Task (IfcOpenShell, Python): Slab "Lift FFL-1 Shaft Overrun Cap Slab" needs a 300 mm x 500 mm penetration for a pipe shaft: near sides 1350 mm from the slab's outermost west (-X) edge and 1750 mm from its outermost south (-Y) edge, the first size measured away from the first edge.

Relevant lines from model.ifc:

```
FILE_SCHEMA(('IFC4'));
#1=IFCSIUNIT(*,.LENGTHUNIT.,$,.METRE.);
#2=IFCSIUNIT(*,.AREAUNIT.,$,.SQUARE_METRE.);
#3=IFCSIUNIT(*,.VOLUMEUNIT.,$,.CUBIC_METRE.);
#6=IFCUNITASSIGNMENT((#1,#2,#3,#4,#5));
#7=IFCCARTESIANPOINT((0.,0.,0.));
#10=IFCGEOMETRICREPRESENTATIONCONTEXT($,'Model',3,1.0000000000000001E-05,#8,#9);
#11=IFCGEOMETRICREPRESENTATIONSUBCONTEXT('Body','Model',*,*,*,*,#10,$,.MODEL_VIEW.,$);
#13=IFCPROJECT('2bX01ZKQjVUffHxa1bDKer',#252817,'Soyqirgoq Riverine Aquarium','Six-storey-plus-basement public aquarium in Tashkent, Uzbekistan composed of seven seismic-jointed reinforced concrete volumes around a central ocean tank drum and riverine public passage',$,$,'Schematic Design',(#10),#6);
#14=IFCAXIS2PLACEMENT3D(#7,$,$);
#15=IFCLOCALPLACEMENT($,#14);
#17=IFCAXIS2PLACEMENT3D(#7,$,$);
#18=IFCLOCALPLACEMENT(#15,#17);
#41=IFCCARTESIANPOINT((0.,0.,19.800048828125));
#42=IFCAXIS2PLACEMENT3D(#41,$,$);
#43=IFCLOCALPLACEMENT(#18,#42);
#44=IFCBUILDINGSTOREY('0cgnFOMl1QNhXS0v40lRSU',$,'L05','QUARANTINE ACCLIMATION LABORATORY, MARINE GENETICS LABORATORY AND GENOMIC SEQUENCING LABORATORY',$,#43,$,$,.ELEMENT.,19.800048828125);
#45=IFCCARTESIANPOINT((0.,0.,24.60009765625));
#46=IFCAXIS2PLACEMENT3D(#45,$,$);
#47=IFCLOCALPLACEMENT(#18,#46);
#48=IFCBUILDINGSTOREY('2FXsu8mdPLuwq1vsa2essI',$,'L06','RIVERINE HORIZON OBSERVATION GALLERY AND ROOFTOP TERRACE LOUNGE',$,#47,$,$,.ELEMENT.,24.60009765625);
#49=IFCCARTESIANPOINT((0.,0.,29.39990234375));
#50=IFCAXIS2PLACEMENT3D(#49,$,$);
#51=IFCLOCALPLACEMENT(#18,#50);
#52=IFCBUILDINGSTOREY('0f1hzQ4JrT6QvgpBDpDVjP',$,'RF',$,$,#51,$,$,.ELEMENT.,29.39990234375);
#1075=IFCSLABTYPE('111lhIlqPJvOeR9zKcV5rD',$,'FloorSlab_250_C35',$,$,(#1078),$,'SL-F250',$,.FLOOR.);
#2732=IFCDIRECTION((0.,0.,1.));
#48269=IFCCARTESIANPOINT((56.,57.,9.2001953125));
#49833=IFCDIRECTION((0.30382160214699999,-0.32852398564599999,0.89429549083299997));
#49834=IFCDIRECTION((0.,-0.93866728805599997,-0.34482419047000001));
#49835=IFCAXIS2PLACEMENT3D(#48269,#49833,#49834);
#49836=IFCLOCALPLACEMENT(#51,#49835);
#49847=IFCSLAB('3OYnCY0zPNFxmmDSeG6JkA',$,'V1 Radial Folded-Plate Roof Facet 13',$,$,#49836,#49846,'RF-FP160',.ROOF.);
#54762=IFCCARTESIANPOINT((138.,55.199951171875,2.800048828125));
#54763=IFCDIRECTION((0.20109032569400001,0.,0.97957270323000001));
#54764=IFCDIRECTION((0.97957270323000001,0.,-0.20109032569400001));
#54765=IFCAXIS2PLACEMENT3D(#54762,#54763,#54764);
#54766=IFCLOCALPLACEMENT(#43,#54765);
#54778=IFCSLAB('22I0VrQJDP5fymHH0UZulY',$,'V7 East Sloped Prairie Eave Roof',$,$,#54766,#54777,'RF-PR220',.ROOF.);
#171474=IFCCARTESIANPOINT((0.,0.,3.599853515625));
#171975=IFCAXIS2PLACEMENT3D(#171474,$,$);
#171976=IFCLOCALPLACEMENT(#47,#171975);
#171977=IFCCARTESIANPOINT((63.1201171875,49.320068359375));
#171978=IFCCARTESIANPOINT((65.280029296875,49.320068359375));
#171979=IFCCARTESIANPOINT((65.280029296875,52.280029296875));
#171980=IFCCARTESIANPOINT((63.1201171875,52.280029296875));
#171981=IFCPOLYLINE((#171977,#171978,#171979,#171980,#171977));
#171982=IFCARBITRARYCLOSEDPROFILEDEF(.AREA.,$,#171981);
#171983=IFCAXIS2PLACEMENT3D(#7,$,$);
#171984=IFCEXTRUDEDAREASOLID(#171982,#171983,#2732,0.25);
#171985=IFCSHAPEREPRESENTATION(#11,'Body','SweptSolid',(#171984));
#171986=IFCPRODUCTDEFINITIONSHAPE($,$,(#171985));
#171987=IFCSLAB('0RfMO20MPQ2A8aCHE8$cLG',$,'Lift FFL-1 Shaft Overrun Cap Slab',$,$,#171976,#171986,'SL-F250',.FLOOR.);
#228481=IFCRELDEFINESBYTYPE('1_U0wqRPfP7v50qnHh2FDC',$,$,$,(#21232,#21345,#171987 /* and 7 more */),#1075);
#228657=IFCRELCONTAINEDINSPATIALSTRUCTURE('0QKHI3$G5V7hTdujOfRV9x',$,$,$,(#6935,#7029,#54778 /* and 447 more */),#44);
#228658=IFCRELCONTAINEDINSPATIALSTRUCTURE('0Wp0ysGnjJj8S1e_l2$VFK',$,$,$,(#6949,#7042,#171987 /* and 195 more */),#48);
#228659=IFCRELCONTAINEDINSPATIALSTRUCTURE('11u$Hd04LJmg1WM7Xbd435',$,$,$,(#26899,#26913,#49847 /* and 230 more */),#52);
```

```python
import numpy as np
import ifcopenshell
import ifcopenshell.api.feature
import ifcopenshell.api.geometry
import ifcopenshell.api.root
import ifcopenshell.geom
import ifcopenshell.util.placement
import ifcopenshell.util.representation
import ifcopenshell.util.shape
import ifcopenshell.util.unit

model = ifcopenshell.open("model.ifc")
unit_scale = ifcopenshell.util.unit.calculate_unit_scale(model)
settings = ifcopenshell.geom.settings()


def volume(element):
    """Net volume in cubic metres, openings subtracted."""
    shape = ifcopenshell.geom.create_shape(settings, element)
    return ifcopenshell.util.shape.get_volume(shape.geometry)


slab = model.by_id(171987)
before = volume(slab)

# Extent in the slab's own axes, in metres. The edges named are its -X and -Y sides.
slab_shape = ifcopenshell.geom.create_shape(settings, slab)
vertices = ifcopenshell.util.shape.get_vertices(slab_shape.geometry)
x_min, y_min, bottom = vertices.min(axis=0)
top = vertices[:, 2].max()

opening = ifcopenshell.api.root.create_entity(model, ifc_class="IfcOpeningElement", name="Pipe shaft opening", predefined_type="OPENING")
context = ifcopenshell.util.representation.get_context(model, "Model", "Body", "MODEL_VIEW")
width, depth = 0.3, 0.5
outline = [(0.0, 0.0), (width, 0.0), (width, depth), (0.0, depth), (0.0, 0.0)]
# Overshoot both faces by 50 mm so the cut is clean.
shape = ifcopenshell.api.geometry.add_slab_representation(
    model, context=context, depth=top - bottom + 0.1, polyline=outline
)
ifcopenshell.api.geometry.assign_representation(model, product=opening, representation=shape)

matrix = ifcopenshell.util.placement.get_local_placement(slab.ObjectPlacement)
matrix[:, 3] = matrix @ np.append(np.array([x_min + 1.35, y_min + 1.75, bottom - 0.05]) / unit_scale, 1.0)
ifcopenshell.api.geometry.edit_object_placement(model, product=opening, matrix=matrix, is_si=False)
ifcopenshell.api.feature.add_feature(model, feature=opening, element=slab)

after = volume(slab)

print(f"slab volume {before:.3f} -> {after:.3f} m3")

model.write("model_v2.ifc")
```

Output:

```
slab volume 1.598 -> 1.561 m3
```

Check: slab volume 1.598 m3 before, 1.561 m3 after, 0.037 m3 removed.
